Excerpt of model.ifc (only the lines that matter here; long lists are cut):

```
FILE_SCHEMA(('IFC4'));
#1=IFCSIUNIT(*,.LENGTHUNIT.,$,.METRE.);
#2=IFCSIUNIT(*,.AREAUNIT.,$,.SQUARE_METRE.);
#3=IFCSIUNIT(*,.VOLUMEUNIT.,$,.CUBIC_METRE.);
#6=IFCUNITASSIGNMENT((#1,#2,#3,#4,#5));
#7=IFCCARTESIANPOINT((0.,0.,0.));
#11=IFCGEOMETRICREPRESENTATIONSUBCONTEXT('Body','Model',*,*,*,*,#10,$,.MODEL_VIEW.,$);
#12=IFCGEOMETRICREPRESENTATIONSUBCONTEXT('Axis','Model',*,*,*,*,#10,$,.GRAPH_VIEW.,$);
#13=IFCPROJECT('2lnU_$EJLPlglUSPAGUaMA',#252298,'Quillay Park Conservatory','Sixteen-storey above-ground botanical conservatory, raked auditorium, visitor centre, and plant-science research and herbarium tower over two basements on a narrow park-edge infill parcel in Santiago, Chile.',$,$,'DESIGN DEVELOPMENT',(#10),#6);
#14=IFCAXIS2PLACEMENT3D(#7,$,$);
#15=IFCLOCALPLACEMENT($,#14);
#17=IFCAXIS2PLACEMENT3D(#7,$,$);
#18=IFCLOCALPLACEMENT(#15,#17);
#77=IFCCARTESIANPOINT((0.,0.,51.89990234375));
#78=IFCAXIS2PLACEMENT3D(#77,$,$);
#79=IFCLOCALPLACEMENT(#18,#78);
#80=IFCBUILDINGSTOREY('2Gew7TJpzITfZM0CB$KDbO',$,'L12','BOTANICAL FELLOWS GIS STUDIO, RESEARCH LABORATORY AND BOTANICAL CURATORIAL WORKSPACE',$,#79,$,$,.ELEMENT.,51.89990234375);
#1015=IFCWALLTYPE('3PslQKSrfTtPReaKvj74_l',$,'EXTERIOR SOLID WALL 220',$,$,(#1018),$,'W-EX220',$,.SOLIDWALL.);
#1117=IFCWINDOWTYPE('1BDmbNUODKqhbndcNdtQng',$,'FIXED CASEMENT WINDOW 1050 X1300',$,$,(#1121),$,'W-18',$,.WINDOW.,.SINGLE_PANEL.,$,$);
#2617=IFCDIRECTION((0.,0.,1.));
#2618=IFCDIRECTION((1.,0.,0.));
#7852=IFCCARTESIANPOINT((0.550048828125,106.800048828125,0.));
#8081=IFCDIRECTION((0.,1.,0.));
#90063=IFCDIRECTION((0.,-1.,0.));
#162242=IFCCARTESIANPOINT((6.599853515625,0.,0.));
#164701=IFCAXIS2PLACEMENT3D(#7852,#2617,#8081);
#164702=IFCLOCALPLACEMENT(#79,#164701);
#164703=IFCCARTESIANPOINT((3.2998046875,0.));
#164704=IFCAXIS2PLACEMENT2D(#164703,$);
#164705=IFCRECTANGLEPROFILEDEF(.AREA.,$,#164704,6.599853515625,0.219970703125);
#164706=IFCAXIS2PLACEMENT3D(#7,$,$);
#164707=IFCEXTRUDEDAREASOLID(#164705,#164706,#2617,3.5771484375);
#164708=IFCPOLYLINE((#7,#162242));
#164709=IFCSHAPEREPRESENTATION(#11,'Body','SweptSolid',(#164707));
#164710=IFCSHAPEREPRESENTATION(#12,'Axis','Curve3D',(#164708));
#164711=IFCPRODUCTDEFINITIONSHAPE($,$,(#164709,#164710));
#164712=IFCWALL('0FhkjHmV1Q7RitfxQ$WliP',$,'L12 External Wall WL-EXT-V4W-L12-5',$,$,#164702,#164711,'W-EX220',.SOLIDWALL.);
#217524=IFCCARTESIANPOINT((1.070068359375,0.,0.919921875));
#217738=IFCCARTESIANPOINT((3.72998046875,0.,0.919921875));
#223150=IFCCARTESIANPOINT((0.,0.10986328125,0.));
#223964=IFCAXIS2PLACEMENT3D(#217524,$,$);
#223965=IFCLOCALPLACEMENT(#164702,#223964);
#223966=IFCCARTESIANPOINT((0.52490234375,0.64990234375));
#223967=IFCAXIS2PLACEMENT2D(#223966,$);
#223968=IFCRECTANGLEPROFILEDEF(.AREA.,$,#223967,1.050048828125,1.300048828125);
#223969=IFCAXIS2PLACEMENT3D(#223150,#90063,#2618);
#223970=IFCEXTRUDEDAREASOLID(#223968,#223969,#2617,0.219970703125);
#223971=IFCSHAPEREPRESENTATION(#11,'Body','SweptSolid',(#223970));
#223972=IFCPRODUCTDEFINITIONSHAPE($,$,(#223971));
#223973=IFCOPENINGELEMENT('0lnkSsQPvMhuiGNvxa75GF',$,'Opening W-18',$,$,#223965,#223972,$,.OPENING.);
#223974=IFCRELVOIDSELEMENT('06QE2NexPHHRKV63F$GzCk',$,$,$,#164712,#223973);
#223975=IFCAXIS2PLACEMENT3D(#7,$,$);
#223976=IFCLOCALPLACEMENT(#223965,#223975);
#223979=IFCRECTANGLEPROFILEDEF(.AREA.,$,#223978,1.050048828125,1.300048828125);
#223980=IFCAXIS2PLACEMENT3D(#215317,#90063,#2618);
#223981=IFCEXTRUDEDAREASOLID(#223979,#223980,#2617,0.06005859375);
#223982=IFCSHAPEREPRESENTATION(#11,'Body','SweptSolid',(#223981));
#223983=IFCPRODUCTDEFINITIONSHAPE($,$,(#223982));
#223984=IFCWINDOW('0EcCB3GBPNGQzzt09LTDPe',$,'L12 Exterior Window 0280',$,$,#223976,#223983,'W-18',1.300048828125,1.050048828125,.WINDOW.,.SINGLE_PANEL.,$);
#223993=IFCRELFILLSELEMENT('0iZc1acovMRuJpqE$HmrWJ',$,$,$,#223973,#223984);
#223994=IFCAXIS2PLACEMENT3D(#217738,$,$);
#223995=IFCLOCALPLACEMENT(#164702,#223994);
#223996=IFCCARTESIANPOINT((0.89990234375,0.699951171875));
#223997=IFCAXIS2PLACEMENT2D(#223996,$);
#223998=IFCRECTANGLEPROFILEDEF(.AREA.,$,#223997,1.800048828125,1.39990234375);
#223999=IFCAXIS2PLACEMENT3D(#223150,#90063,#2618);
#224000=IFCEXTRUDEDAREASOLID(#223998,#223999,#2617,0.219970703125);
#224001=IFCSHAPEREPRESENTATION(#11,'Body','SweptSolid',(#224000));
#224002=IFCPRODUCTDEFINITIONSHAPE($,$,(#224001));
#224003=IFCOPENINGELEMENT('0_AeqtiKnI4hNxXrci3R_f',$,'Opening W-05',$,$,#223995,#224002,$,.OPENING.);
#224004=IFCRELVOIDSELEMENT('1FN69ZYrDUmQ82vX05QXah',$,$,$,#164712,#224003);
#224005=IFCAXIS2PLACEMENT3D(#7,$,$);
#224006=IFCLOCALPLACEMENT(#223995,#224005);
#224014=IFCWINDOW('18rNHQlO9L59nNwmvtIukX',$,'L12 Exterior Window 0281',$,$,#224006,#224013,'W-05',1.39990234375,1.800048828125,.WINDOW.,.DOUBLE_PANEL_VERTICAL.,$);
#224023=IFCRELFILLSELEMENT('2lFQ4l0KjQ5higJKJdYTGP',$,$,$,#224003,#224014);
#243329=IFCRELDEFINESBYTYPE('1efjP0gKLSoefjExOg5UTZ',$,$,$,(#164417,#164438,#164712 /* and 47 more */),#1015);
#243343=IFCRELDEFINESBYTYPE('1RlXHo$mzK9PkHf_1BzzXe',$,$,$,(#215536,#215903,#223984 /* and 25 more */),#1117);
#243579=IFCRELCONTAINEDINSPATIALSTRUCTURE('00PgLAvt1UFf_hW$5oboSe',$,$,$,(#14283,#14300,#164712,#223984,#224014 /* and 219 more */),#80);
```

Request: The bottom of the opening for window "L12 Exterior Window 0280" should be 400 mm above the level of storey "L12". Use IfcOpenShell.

```python
import numpy as np
import ifcopenshell
import ifcopenshell.api.geometry
import ifcopenshell.geom
import ifcopenshell.util.element
import ifcopenshell.util.placement
import ifcopenshell.util.shape
import ifcopenshell.util.unit

model = ifcopenshell.open("model.ifc")
unit_scale = ifcopenshell.util.unit.calculate_unit_scale(model)

window = model.by_id(223984)
opening = window.FillsVoids[0].RelatingOpeningElement
storey = ifcopenshell.util.element.get_container(window, ifc_class="IfcBuildingStorey")
level = ifcopenshell.util.placement.get_local_placement(storey.ObjectPlacement)[2, 3]

# The opening's origin need not be at the sill, so measure its lowest point.
shape = ifcopenshell.geom.create_shape(ifcopenshell.geom.settings(), opening)
bottom = ifcopenshell.util.shape.get_shape_bottom_elevation(shape, shape.geometry) / unit_scale
dz = level + 0.4 - bottom

shift = np.array([0.0, 0.0, dz])
# The window is placed relative to its opening, so it follows when the opening moves.
matrix = ifcopenshell.util.placement.get_local_placement(opening.ObjectPlacement)
matrix[:3, 3] += shift
ifcopenshell.api.geometry.edit_object_placement(
    model, product=opening, matrix=matrix, is_si=False, should_transform_children=True
)

print(f"moved by {dz * unit_scale:+.3f} m")

model.write("model_v2.ifc")
```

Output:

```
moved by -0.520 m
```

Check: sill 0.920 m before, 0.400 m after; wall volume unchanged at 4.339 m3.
